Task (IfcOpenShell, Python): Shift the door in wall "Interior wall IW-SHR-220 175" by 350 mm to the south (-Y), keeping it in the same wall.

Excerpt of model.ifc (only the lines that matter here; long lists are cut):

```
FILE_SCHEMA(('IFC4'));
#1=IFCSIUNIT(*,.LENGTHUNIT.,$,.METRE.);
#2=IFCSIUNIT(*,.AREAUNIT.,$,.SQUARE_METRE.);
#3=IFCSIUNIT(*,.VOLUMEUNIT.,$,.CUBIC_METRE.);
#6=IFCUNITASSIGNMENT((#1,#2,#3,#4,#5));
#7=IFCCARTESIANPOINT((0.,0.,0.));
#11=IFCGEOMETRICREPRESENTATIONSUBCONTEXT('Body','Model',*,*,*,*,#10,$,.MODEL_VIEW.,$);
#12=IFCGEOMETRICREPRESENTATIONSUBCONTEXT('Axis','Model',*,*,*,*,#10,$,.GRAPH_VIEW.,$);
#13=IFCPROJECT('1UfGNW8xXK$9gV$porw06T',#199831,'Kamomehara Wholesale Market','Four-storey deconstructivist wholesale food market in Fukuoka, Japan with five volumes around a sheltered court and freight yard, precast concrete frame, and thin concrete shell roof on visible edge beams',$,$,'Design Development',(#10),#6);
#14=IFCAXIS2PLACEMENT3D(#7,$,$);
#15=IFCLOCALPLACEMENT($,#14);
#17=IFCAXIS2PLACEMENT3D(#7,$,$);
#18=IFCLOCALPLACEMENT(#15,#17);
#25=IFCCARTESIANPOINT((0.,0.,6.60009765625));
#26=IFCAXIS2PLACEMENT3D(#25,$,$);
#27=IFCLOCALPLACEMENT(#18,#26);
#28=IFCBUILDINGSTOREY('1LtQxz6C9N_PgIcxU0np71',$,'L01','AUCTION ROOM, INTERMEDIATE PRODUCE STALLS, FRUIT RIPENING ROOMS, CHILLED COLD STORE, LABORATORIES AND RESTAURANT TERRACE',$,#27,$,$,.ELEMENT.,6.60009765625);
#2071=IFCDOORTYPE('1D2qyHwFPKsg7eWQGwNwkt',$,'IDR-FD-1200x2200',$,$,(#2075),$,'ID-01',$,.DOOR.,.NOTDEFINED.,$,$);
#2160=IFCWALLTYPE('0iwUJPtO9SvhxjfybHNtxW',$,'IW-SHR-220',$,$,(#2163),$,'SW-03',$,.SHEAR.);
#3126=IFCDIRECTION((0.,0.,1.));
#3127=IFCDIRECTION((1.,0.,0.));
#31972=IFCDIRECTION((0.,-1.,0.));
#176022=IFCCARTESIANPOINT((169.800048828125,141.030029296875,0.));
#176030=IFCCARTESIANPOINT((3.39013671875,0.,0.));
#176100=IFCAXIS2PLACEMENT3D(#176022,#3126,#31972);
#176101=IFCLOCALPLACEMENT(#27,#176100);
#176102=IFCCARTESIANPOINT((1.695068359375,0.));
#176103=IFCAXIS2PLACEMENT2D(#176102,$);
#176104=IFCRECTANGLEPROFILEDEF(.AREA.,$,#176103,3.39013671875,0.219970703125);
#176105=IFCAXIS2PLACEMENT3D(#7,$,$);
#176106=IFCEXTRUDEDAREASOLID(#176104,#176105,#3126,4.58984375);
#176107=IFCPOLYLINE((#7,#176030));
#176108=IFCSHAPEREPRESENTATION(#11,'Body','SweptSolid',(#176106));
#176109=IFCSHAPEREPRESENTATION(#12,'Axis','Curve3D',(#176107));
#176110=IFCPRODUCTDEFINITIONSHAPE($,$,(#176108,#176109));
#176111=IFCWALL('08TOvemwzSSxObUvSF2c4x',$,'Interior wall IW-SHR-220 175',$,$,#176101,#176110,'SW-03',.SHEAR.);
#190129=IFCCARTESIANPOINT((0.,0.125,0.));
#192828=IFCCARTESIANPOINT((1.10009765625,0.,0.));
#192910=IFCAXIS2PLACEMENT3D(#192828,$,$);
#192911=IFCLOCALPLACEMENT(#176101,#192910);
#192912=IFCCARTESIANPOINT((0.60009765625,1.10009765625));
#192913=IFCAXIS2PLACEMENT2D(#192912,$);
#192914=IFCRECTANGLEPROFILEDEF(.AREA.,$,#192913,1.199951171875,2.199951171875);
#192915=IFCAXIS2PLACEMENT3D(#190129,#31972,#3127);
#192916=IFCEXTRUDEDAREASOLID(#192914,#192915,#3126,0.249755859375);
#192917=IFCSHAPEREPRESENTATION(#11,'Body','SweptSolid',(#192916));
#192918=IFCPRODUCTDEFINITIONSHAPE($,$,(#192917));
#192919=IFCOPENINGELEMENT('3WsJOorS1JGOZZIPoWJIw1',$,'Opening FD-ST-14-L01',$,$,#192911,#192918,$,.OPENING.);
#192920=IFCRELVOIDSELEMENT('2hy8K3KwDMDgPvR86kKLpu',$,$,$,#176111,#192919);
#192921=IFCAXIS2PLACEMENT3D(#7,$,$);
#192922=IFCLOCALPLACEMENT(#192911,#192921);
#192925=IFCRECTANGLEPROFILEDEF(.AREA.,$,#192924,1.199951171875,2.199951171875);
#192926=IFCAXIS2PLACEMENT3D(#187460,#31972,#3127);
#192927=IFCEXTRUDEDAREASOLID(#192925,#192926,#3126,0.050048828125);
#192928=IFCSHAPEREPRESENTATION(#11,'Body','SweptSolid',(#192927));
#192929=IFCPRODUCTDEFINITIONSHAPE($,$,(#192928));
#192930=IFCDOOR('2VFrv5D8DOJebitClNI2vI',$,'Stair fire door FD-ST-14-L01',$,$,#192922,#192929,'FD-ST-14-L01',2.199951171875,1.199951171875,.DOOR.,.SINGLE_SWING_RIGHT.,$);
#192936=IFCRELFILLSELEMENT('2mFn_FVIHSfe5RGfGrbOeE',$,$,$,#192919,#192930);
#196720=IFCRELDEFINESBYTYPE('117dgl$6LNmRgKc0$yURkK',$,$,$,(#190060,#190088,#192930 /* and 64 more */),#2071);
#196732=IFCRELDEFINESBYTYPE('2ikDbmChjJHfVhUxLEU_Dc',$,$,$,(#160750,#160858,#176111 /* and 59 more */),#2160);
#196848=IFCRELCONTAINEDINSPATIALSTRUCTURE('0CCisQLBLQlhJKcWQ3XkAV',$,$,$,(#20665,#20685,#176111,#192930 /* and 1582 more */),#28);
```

```python
import ifcopenshell
import ifcopenshell.api.geometry
import ifcopenshell.util.placement

model = ifcopenshell.open("model.ifc")

door = model.by_id(192930)
opening = door.FillsVoids[0].RelatingOpeningElement
wall = opening.VoidsElements[0].RelatingBuildingElement

wall_matrix = ifcopenshell.util.placement.get_local_placement(wall.ObjectPlacement)
shift = wall_matrix[:3, 0] * 0.35
before = ifcopenshell.util.placement.get_local_placement(door.ObjectPlacement)[:3, 3].copy()

# The door is placed relative to its opening, so it follows when the opening moves.
matrix = ifcopenshell.util.placement.get_local_placement(opening.ObjectPlacement)
matrix[:3, 3] += shift
ifcopenshell.api.geometry.edit_object_placement(
    model, product=opening, matrix=matrix, is_si=False, should_transform_children=True
)

after = ifcopenshell.util.placement.get_local_placement(door.ObjectPlacement)[:3, 3]
print("door moved by", (after - before).round(3) + 0.0)

model.write("model_v2.ifc")
```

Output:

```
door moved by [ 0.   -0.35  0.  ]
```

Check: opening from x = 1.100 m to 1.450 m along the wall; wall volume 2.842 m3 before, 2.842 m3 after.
